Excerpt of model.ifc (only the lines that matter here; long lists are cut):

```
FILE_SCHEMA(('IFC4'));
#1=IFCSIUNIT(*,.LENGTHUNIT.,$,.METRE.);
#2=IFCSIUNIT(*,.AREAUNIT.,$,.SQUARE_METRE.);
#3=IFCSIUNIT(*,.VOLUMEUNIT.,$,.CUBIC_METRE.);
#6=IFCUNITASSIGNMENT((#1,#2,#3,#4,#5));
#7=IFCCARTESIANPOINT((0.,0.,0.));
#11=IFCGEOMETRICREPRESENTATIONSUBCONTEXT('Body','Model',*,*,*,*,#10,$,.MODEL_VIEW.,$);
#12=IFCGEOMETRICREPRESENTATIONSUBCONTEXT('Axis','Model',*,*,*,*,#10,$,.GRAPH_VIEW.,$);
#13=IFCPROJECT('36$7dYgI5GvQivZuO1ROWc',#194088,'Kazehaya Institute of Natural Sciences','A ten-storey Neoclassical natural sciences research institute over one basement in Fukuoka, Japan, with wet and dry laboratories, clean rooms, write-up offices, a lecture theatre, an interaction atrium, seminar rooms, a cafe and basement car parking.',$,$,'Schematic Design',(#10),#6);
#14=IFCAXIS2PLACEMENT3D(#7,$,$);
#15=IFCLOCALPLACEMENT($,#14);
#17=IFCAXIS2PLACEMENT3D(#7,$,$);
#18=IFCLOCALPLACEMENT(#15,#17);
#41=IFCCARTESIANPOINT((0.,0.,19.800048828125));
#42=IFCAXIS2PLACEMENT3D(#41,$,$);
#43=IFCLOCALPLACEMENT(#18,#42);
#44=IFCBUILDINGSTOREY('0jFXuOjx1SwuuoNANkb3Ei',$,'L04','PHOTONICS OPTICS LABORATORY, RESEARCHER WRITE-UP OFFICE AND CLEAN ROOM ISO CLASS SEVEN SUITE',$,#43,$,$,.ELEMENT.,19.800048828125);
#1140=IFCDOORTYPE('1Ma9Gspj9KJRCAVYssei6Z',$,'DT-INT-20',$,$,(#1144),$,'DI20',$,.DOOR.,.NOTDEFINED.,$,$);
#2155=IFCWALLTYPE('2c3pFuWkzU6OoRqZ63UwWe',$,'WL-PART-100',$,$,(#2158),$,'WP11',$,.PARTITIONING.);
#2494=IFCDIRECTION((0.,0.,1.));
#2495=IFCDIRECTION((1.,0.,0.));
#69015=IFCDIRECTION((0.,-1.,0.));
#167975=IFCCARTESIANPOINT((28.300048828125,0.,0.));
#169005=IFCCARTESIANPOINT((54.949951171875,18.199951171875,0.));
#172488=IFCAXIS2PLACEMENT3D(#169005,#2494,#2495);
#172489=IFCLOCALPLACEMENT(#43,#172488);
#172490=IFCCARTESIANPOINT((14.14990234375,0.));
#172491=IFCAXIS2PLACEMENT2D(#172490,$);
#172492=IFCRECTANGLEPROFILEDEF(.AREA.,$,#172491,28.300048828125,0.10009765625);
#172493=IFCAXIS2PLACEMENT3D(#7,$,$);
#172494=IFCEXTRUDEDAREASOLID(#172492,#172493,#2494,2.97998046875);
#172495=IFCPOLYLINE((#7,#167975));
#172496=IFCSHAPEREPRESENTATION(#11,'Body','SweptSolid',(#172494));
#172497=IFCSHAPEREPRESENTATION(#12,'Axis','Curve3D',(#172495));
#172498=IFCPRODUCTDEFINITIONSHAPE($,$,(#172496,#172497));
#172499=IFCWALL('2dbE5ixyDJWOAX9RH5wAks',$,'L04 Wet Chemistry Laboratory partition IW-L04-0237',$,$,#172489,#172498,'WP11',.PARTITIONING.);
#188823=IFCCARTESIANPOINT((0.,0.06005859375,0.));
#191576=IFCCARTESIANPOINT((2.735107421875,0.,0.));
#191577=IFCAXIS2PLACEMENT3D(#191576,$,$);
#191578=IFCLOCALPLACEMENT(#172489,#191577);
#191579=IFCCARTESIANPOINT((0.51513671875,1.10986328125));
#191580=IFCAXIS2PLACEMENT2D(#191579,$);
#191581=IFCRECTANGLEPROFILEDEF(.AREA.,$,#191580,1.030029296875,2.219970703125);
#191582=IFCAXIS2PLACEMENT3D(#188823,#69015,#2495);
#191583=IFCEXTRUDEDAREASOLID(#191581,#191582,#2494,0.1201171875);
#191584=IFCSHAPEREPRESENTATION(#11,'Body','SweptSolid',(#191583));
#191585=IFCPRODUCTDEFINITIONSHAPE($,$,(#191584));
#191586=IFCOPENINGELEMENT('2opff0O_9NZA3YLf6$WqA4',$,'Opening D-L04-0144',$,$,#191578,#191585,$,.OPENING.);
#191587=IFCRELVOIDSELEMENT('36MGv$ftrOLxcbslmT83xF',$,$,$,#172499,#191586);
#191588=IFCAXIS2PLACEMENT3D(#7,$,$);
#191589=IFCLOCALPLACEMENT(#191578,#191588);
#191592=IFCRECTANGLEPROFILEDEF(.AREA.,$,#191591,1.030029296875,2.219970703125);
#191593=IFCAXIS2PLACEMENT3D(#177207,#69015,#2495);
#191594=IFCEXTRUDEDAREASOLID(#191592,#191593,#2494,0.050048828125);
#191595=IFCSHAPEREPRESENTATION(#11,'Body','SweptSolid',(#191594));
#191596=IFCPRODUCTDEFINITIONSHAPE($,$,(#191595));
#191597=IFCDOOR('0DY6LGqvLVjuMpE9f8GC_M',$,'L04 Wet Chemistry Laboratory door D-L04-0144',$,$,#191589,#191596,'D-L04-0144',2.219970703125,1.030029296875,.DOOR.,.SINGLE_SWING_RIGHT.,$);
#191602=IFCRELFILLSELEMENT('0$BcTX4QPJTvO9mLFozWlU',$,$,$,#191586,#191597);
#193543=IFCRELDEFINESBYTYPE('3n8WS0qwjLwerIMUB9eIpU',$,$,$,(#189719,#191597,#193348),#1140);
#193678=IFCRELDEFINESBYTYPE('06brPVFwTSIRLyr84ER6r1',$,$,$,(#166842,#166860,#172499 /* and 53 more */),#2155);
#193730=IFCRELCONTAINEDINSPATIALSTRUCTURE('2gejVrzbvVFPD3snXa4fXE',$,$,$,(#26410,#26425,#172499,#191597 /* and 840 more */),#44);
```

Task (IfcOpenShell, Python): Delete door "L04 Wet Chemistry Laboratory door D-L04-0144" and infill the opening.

```python
import ifcopenshell
import ifcopenshell.api.feature
import ifcopenshell.api.root
import ifcopenshell.geom
import ifcopenshell.util.shape

model = ifcopenshell.open("model.ifc")
settings = ifcopenshell.geom.settings()


def volume(element):
    """Net volume in cubic metres, openings subtracted."""
    shape = ifcopenshell.geom.create_shape(settings, element)
    return ifcopenshell.util.shape.get_volume(shape.geometry)


door = model.by_guid("0DY6LGqvLVjuMpE9f8GC_M")
opening = door.FillsVoids[0].RelatingOpeningElement
wall = opening.VoidsElements[0].RelatingBuildingElement
before = volume(wall)

ifcopenshell.api.root.remove_product(model, product=door)
ifcopenshell.api.feature.remove_feature(model, feature=opening)

after = volume(wall)

print(f"wall volume {before:.3f} -> {after:.3f} m3")

model.write("model_v2.ifc")
```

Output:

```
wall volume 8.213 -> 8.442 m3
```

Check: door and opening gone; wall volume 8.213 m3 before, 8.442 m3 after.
